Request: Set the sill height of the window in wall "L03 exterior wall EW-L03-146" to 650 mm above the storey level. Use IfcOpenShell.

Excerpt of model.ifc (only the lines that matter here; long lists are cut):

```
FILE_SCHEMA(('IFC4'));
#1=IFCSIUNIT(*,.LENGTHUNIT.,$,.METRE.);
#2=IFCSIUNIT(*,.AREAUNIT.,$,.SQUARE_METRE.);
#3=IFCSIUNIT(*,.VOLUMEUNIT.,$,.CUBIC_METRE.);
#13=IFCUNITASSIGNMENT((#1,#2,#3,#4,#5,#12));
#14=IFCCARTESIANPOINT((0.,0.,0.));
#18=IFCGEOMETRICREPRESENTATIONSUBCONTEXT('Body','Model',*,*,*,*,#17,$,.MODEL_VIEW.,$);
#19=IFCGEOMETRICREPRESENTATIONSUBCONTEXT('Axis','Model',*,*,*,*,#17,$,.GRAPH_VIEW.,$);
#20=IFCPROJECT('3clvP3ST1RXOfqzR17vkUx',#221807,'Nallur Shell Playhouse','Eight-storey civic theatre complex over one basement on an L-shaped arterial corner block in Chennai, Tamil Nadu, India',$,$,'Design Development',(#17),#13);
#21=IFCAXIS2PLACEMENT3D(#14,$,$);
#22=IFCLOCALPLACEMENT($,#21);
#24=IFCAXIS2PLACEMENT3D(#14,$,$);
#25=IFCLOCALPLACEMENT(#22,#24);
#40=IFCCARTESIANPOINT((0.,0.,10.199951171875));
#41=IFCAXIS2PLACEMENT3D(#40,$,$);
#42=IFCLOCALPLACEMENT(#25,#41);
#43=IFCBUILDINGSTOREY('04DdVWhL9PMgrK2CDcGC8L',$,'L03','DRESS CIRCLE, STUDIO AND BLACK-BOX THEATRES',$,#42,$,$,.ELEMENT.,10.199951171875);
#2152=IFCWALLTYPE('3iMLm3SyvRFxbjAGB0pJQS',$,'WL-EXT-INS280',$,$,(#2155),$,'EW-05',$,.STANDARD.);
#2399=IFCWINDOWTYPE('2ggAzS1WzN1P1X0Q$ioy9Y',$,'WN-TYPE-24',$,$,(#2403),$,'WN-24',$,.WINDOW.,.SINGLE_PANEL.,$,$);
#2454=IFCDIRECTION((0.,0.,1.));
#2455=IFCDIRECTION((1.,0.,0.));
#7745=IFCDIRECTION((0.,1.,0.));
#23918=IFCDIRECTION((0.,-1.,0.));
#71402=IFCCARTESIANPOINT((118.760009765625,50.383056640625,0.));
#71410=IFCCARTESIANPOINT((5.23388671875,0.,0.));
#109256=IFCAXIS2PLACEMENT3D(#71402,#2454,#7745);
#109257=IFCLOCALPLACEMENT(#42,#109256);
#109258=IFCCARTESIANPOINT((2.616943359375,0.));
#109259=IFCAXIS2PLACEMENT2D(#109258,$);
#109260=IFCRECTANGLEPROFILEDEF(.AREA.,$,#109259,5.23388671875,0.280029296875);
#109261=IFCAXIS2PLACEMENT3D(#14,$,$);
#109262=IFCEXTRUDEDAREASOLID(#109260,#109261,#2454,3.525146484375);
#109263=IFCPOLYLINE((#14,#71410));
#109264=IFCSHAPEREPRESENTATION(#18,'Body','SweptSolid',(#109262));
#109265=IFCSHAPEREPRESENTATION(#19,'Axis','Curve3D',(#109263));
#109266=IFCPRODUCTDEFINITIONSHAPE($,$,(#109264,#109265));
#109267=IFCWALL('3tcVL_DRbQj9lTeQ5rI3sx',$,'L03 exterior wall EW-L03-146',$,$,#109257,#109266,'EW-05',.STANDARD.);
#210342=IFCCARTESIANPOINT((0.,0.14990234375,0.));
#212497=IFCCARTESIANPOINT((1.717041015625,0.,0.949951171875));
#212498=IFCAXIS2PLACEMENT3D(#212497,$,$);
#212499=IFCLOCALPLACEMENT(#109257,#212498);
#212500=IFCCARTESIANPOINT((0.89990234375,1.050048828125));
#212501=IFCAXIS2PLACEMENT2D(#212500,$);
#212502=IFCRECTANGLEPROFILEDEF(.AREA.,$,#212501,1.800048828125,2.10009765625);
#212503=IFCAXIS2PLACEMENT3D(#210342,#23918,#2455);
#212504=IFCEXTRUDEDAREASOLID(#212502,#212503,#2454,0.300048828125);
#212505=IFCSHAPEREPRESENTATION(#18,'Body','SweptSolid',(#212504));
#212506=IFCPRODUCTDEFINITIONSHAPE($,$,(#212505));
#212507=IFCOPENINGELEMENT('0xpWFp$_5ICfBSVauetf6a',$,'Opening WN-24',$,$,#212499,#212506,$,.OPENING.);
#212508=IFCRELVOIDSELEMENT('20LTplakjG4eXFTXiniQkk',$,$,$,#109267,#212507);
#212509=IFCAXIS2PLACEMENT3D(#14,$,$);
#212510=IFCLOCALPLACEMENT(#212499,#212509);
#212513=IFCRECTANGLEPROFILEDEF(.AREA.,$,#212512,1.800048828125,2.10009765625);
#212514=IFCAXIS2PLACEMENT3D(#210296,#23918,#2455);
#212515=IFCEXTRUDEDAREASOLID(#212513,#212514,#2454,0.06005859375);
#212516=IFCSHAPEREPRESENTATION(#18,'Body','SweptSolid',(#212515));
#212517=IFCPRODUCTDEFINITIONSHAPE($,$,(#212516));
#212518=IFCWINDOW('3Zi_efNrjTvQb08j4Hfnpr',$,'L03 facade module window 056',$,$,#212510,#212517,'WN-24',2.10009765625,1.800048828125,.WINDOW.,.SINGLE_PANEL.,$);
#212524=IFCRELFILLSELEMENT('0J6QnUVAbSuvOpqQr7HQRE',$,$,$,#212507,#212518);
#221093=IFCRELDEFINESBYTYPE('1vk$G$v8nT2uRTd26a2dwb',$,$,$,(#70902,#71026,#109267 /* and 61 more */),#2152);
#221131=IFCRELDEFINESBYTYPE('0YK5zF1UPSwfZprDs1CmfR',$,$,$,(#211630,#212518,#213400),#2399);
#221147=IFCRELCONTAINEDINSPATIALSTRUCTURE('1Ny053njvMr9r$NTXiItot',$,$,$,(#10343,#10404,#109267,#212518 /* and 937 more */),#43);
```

```python
import numpy as np
import ifcopenshell
import ifcopenshell.api.geometry
import ifcopenshell.geom
import ifcopenshell.util.element
import ifcopenshell.util.placement
import ifcopenshell.util.shape
import ifcopenshell.util.unit

model = ifcopenshell.open("model.ifc")
unit_scale = ifcopenshell.util.unit.calculate_unit_scale(model)

window = model.by_id(212518)
opening = window.FillsVoids[0].RelatingOpeningElement
storey = ifcopenshell.util.element.get_container(window, ifc_class="IfcBuildingStorey")
level = ifcopenshell.util.placement.get_local_placement(storey.ObjectPlacement)[2, 3]

# The opening's origin need not be at the sill, so measure its lowest point.
shape = ifcopenshell.geom.create_shape(ifcopenshell.geom.settings(), opening)
bottom = ifcopenshell.util.shape.get_shape_bottom_elevation(shape, shape.geometry) / unit_scale
dz = level + 0.65 / unit_scale - bottom

shift = np.array([0.0, 0.0, dz])
# The window is placed relative to its opening, so it follows when the opening moves.
matrix = ifcopenshell.util.placement.get_local_placement(opening.ObjectPlacement)
matrix[:3, 3] += shift
ifcopenshell.api.geometry.edit_object_placement(
    model, product=opening, matrix=matrix, is_si=False, should_transform_children=True
)

print(f"moved by {dz * unit_scale:+.3f} m")

model.write("model_v2.ifc")
```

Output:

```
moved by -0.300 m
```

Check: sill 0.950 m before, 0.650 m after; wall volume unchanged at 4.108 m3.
